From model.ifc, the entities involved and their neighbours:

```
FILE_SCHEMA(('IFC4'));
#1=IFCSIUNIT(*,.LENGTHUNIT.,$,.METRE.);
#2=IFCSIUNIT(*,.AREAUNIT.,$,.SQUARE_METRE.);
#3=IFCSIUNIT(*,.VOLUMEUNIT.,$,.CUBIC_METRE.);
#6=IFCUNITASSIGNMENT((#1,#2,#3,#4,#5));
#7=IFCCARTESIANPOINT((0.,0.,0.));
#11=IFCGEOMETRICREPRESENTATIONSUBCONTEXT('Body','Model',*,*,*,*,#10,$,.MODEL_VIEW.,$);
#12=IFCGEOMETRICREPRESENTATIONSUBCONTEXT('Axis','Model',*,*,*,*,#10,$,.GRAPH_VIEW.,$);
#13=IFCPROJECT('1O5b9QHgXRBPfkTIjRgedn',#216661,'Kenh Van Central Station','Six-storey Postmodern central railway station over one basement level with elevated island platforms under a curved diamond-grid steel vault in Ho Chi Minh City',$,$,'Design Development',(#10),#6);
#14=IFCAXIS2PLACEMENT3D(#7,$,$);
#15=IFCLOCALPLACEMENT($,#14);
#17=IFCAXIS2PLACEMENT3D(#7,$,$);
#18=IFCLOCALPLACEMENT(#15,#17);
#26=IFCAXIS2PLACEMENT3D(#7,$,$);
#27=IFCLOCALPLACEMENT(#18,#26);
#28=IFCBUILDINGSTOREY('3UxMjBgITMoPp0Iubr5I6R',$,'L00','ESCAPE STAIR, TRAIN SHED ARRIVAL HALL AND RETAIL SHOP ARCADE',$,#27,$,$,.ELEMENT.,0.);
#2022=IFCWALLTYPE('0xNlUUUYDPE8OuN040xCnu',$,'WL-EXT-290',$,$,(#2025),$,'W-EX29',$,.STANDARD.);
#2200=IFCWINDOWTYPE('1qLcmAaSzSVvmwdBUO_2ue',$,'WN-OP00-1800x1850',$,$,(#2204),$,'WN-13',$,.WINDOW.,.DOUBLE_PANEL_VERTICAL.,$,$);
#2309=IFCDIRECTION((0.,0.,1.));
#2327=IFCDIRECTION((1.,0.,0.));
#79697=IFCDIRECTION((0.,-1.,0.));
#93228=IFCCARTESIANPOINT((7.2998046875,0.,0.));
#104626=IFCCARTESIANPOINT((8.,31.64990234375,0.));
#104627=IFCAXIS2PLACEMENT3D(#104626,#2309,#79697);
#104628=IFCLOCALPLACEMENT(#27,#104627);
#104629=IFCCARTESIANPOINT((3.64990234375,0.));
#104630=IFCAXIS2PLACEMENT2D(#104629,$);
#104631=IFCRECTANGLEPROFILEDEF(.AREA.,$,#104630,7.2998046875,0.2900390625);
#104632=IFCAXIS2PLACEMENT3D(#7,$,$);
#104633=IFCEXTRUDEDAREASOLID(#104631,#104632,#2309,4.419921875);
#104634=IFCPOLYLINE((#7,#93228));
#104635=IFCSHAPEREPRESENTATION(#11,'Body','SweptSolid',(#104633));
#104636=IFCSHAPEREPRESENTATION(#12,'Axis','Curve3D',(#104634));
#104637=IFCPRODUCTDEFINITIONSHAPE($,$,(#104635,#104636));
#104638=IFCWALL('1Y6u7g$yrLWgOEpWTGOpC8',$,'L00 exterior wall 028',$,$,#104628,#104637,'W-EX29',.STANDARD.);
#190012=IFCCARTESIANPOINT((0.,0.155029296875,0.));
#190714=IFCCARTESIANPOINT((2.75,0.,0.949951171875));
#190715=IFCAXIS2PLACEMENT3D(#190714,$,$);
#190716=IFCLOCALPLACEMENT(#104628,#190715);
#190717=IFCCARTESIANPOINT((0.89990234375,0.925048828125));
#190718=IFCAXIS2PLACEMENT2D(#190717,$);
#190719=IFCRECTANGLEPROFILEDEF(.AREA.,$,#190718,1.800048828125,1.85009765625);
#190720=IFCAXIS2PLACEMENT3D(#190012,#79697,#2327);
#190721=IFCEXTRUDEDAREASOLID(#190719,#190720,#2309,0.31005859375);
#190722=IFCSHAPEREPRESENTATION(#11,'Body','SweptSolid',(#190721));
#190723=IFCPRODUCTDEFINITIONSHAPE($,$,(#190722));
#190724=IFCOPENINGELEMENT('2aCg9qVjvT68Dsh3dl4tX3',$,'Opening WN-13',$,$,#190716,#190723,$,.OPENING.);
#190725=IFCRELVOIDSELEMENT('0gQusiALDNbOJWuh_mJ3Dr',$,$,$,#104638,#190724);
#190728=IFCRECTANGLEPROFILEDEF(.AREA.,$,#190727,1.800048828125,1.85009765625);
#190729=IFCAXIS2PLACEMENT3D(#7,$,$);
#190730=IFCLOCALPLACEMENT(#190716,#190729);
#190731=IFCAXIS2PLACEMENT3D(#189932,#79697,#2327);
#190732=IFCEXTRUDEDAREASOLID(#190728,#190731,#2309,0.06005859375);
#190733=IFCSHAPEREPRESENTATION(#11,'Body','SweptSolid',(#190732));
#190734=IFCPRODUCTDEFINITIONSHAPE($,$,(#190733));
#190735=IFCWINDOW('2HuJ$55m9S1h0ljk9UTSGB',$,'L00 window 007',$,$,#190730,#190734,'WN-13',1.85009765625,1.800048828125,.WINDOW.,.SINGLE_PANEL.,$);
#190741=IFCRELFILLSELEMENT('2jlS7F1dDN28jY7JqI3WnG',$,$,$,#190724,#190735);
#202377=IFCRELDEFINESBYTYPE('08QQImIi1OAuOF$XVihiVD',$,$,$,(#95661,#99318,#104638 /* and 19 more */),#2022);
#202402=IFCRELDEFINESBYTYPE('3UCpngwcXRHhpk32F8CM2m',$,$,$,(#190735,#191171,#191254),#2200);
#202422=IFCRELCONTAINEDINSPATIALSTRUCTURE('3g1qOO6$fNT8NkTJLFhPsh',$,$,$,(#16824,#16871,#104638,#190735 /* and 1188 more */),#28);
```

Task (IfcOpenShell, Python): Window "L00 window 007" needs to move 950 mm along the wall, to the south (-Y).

```python
import ifcopenshell
import ifcopenshell.api.geometry
import ifcopenshell.util.placement

model = ifcopenshell.open("model.ifc")

window = model.by_guid("2HuJ$55m9S1h0ljk9UTSGB")
opening = window.FillsVoids[0].RelatingOpeningElement
wall = opening.VoidsElements[0].RelatingBuildingElement

wall_matrix = ifcopenshell.util.placement.get_local_placement(wall.ObjectPlacement)
shift = wall_matrix[:3, 0] * 0.95
before = ifcopenshell.util.placement.get_local_placement(window.ObjectPlacement)[:3, 3].copy()

# The window is placed relative to its opening, so it follows when the opening moves.
matrix = ifcopenshell.util.placement.get_local_placement(opening.ObjectPlacement)
matrix[:3, 3] += shift
ifcopenshell.api.geometry.edit_object_placement(
    model, product=opening, matrix=matrix, is_si=False, should_transform_children=True
)

after = ifcopenshell.util.placement.get_local_placement(window.ObjectPlacement)[:3, 3]
print("window moved by", (after - before).round(3) + 0.0)

model.write("model_edited.ifc")
```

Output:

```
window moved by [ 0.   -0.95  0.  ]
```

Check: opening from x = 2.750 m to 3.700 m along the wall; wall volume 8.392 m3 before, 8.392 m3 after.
